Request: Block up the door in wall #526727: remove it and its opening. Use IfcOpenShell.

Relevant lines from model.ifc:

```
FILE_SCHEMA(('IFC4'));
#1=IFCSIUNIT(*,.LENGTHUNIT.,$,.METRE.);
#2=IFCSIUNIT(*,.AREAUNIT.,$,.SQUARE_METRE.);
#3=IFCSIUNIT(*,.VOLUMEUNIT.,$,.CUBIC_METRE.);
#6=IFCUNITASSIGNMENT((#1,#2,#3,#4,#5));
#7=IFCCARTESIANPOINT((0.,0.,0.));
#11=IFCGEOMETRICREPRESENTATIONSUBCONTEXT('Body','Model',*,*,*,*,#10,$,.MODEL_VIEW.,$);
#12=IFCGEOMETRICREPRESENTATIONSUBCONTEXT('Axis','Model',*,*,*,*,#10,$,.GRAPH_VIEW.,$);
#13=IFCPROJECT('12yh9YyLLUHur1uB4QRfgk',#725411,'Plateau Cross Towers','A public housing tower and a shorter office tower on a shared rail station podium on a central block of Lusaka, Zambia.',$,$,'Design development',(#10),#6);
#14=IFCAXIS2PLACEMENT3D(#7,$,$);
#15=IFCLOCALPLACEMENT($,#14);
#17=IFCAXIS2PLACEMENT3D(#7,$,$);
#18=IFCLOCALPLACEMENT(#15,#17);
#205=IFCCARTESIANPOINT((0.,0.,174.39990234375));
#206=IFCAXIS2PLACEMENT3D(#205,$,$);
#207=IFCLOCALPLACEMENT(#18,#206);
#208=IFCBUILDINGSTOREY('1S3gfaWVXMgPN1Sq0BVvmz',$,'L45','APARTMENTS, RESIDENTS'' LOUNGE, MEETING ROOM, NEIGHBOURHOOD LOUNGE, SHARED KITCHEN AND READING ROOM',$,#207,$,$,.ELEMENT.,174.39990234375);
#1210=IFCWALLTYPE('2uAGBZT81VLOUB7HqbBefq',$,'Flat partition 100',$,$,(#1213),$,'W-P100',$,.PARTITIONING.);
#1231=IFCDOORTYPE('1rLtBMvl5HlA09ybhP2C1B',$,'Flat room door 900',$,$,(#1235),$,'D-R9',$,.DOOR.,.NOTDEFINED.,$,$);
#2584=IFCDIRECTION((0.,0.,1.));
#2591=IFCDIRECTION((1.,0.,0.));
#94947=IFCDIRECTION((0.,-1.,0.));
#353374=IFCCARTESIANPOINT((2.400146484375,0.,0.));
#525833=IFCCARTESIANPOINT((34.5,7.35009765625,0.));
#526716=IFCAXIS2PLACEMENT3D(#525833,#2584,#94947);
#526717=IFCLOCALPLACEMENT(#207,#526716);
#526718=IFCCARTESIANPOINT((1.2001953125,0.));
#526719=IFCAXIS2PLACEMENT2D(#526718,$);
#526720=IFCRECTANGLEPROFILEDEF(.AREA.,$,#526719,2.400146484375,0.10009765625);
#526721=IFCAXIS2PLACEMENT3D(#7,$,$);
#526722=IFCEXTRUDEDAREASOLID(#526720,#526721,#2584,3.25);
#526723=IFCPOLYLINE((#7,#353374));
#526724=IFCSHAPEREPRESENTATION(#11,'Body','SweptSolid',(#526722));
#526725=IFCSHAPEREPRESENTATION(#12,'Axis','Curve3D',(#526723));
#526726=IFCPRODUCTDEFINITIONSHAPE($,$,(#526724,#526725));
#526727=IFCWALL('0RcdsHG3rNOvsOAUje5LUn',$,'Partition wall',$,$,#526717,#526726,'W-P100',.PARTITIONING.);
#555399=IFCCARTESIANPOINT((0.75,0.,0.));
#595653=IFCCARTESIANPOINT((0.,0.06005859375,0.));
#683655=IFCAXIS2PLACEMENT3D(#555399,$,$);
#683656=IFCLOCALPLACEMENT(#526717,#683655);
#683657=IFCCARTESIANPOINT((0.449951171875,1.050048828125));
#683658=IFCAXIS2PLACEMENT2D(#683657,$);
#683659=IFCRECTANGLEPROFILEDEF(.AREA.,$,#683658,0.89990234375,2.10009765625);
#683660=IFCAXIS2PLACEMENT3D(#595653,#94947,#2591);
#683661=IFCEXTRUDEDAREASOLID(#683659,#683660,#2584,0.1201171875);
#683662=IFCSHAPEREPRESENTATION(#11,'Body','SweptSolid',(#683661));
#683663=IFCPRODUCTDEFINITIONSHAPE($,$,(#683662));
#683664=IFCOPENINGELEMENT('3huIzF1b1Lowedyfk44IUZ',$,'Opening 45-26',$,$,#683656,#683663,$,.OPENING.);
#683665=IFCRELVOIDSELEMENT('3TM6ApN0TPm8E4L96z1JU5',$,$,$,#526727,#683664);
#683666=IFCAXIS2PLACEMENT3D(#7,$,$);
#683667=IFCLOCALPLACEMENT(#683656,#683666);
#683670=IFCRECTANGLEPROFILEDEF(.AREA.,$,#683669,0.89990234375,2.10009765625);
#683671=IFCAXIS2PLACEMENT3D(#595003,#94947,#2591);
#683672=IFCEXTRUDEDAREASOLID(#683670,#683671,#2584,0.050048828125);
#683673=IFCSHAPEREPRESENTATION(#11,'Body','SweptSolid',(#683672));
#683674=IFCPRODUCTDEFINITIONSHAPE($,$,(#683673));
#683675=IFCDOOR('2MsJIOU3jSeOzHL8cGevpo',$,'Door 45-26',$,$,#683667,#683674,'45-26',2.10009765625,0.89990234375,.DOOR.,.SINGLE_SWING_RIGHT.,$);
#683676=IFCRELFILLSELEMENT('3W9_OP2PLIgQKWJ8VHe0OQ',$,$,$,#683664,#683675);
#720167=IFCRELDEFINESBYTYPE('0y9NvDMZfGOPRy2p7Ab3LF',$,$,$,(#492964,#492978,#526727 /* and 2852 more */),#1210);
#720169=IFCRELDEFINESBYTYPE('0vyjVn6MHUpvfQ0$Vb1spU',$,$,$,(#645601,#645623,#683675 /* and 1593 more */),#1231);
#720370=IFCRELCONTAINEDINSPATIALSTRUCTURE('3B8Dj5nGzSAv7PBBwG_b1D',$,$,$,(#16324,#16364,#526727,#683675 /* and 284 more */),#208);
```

```python
import ifcopenshell
import ifcopenshell.api.feature
import ifcopenshell.api.root
import ifcopenshell.geom
import ifcopenshell.util.shape

model = ifcopenshell.open("model.ifc")
settings = ifcopenshell.geom.settings()


def volume(element):
    """Net volume in cubic metres, openings subtracted."""
    shape = ifcopenshell.geom.create_shape(settings, element)
    return ifcopenshell.util.shape.get_volume(shape.geometry)


door = model.by_guid("2MsJIOU3jSeOzHL8cGevpo")
opening = door.FillsVoids[0].RelatingOpeningElement
wall = opening.VoidsElements[0].RelatingBuildingElement
before = volume(wall)

ifcopenshell.api.root.remove_product(model, product=door)
ifcopenshell.api.feature.remove_feature(model, feature=opening)

after = volume(wall)

print(f"wall volume {before:.3f} -> {after:.3f} m3")

model.write("model_rev.ifc")
```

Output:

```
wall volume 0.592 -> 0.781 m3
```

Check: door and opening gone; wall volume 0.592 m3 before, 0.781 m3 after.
